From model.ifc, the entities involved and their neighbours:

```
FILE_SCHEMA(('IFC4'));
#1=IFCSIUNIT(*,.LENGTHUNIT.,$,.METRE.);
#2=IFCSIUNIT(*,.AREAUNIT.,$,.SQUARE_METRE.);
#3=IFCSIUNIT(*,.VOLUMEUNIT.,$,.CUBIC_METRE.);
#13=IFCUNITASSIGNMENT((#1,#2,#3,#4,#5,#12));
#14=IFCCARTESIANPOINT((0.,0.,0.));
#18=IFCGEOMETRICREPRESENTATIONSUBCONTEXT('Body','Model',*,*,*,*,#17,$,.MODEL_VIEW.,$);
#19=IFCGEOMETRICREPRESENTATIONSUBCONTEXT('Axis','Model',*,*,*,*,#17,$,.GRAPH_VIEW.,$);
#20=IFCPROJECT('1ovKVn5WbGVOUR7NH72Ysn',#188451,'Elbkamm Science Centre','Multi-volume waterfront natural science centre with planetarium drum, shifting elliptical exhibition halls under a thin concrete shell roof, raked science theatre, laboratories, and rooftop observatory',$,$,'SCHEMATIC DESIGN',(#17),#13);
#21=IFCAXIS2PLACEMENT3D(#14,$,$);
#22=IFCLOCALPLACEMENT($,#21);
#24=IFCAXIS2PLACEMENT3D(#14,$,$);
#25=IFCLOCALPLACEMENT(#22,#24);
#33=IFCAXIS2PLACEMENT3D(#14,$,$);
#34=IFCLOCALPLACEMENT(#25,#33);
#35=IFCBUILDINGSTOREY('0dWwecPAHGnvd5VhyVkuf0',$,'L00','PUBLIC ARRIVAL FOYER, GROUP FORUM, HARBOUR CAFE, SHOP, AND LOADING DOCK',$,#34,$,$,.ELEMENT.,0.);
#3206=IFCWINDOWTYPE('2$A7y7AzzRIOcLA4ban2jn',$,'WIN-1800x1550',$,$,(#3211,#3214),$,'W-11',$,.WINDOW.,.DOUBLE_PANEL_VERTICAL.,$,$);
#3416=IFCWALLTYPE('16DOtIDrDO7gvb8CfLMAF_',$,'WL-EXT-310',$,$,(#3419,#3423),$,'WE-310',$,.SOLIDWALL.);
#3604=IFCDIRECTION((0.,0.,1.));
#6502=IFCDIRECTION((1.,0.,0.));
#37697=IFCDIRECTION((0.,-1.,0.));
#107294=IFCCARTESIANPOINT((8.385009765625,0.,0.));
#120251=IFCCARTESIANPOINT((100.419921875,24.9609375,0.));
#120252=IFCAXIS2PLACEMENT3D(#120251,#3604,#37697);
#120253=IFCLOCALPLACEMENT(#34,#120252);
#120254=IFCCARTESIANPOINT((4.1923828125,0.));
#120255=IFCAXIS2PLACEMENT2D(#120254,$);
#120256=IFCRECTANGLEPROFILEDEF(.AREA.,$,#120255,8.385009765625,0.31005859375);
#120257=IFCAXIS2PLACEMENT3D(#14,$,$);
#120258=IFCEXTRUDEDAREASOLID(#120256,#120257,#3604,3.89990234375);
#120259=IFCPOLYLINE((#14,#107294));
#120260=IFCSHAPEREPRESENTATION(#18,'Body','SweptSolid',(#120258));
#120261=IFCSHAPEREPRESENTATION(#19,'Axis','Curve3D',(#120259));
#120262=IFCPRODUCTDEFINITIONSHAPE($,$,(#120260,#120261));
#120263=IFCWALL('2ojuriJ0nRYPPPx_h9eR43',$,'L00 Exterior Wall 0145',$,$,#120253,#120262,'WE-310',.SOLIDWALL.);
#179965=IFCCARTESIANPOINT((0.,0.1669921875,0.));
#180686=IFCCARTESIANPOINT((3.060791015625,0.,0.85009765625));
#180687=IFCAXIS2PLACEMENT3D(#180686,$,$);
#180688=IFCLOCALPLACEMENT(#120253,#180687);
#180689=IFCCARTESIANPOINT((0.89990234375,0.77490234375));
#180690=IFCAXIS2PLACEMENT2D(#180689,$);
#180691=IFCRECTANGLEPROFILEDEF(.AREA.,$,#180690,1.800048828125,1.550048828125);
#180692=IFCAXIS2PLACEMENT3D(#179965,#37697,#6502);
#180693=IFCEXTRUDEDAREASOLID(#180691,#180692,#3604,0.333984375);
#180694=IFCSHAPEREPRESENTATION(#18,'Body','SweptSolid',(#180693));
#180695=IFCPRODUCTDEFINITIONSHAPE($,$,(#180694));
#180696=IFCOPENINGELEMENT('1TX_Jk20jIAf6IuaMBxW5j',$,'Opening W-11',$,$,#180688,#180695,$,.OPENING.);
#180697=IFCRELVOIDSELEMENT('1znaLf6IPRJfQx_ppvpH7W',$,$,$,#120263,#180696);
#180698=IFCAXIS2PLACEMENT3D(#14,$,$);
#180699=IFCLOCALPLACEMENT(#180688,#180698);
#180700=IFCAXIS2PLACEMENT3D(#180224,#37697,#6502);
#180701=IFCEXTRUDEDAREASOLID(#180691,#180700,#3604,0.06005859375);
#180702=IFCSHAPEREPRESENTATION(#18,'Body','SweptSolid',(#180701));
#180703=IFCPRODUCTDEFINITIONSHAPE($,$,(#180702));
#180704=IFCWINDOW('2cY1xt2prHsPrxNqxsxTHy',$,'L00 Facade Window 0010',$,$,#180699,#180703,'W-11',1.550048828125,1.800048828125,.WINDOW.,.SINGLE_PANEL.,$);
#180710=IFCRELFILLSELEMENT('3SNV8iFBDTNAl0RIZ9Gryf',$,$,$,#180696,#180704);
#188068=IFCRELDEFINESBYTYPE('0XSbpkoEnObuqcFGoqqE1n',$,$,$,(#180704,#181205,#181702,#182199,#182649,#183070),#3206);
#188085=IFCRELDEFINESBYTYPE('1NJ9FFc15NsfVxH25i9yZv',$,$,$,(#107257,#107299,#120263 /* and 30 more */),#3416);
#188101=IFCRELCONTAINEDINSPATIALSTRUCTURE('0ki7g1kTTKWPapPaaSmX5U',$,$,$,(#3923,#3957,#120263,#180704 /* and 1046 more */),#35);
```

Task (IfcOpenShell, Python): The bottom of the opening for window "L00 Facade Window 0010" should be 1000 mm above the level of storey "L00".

```python
import numpy as np
import ifcopenshell
import ifcopenshell.api.geometry
import ifcopenshell.geom
import ifcopenshell.util.element
import ifcopenshell.util.placement
import ifcopenshell.util.shape
import ifcopenshell.util.unit

model = ifcopenshell.open("model.ifc")
unit_scale = ifcopenshell.util.unit.calculate_unit_scale(model)

window = model.by_id(180704)
opening = window.FillsVoids[0].RelatingOpeningElement
storey = ifcopenshell.util.element.get_container(window, ifc_class="IfcBuildingStorey")
level = ifcopenshell.util.placement.get_local_placement(storey.ObjectPlacement)[2, 3]

# The opening's origin need not be at the sill, so measure its lowest point.
shape = ifcopenshell.geom.create_shape(ifcopenshell.geom.settings(), opening)
bottom = ifcopenshell.util.shape.get_shape_bottom_elevation(shape, shape.geometry) / unit_scale
dz = level + 1 / unit_scale - bottom

shift = np.array([0.0, 0.0, dz])
# The window is placed relative to its opening, so it follows when the opening moves.
matrix = ifcopenshell.util.placement.get_local_placement(opening.ObjectPlacement)
matrix[:3, 3] += shift
ifcopenshell.api.geometry.edit_object_placement(
    model, product=opening, matrix=matrix, is_si=False, should_transform_children=True
)

print(f"moved by {dz * unit_scale:+.3f} m")

model.write("model_rev.ifc")
```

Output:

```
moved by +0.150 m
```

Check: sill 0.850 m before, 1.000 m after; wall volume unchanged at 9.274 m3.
